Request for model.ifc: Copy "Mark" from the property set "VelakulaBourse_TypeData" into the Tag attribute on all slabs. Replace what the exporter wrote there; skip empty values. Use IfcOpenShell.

First a look at what the model holds.

```python
import ifcopenshell
import ifcopenshell.util.element

model = ifcopenshell.open("model.ifc")
print(model.schema)
slabs = model.by_type("IfcSlab")
print(len(slabs), "slabs")
for e in slabs[:8]:
    source = ifcopenshell.util.element.get_pset(e, "VelakulaBourse_TypeData", "Mark")
    target = e.Tag
    print(e.id(), repr(source), repr(target), sep=" | ")
```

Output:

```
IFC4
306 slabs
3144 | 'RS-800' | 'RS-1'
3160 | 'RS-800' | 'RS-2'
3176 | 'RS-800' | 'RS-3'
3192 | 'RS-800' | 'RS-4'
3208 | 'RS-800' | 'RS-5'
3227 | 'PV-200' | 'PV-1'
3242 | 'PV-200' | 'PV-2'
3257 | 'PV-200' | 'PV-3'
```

```python
import ifcopenshell
import ifcopenshell.util.element

model = ifcopenshell.open("model.ifc")

count = 0
for e in model.by_type("IfcSlab"):
    value = ifcopenshell.util.element.get_pset(e, "VelakulaBourse_TypeData", "Mark")
    current = e.Tag
    if not value or not value.strip() or current == value:
        continue
    e.Tag = value
    count += 1

print(count, "slabs updated")

model.write("model_edited.ifc")
```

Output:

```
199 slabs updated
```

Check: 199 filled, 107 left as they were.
